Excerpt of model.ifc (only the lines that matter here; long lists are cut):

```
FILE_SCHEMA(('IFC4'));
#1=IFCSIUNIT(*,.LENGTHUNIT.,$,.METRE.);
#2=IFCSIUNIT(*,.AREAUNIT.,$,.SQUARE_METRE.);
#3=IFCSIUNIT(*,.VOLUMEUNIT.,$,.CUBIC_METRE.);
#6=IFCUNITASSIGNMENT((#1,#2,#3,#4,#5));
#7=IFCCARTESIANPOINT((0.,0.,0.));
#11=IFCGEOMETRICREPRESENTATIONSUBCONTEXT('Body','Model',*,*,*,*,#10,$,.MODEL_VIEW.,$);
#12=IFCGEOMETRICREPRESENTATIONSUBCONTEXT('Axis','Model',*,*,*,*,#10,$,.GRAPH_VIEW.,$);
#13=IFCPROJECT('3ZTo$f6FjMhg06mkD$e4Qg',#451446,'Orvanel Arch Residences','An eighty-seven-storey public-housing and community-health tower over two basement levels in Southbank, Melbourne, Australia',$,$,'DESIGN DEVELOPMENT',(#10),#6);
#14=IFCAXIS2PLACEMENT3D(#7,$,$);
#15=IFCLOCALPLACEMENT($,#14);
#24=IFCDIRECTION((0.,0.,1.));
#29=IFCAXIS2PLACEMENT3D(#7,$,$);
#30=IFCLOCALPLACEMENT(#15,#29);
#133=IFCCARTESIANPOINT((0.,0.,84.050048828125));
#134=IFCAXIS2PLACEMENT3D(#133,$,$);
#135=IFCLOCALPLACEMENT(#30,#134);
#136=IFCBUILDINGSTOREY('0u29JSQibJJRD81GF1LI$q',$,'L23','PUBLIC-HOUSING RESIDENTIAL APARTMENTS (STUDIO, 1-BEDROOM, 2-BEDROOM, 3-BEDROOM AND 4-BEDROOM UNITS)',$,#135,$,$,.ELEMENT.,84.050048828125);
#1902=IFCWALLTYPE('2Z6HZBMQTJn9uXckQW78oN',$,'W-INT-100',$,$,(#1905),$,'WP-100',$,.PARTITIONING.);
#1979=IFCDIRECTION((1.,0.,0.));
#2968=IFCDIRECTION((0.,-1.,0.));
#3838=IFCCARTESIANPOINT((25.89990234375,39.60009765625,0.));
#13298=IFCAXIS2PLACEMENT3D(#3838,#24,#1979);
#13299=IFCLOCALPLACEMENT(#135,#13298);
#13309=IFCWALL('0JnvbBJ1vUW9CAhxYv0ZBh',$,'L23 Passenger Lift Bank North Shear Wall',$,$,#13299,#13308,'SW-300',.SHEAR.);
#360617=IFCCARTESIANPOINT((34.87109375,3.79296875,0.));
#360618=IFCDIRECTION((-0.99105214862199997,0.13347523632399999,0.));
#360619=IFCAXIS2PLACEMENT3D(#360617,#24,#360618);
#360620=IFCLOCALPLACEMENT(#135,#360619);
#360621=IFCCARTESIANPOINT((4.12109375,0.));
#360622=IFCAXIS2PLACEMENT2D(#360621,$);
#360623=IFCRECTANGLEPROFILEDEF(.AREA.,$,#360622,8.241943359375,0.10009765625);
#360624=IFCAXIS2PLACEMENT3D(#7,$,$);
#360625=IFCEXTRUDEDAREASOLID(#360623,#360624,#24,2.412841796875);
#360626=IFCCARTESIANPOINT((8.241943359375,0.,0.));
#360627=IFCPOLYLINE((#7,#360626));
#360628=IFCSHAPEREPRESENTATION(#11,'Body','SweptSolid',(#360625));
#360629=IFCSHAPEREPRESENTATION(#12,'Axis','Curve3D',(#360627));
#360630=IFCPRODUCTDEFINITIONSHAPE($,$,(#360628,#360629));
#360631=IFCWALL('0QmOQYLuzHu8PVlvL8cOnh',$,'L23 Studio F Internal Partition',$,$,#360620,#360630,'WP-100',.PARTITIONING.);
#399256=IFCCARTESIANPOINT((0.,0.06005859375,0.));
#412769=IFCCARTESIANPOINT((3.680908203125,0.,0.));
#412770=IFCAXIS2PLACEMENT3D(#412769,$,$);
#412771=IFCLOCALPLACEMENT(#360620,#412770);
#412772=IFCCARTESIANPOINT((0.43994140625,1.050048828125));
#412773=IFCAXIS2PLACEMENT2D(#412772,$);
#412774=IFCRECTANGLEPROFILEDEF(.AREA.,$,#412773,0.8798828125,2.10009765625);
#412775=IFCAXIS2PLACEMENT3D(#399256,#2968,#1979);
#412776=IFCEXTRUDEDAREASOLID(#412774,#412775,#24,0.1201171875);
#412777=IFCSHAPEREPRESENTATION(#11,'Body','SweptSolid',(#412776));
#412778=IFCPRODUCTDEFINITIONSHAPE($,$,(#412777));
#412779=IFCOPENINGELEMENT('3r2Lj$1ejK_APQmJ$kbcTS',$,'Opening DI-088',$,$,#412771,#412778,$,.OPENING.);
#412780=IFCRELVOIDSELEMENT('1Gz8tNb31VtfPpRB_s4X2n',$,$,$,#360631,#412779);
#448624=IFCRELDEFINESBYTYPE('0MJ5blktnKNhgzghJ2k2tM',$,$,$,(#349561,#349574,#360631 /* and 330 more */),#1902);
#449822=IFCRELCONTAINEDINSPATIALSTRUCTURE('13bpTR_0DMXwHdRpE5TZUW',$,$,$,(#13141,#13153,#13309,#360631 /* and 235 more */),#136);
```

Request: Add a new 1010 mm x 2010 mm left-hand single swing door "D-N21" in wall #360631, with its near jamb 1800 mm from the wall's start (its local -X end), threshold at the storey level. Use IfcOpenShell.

```python
import numpy as np
import ifcopenshell
import ifcopenshell.api.feature
import ifcopenshell.api.geometry
import ifcopenshell.api.root
import ifcopenshell.api.spatial
import ifcopenshell.geom
import ifcopenshell.util.element
import ifcopenshell.util.placement
import ifcopenshell.util.representation
import ifcopenshell.util.shape
import ifcopenshell.util.unit

model = ifcopenshell.open("model.ifc")
unit_scale = ifcopenshell.util.unit.calculate_unit_scale(model)
settings = ifcopenshell.geom.settings()


def volume(element):
    """Net volume in cubic metres, openings subtracted."""
    shape = ifcopenshell.geom.create_shape(settings, element)
    return ifcopenshell.util.shape.get_volume(shape.geometry)


wall = model.by_guid("0QmOQYLuzHu8PVlvL8cOnh")
storey = ifcopenshell.util.element.get_container(wall, ifc_class="IfcBuildingStorey")
context = ifcopenshell.util.representation.get_context(model, "Model", "Body", "MODEL_VIEW")
before = volume(wall)

width, height, from_end, sill = 1.01, 2.01, 1.8, 0.0  # metres

# The wall runs along its own X axis, and the end named is its -X end.
wall_shape = ifcopenshell.geom.create_shape(settings, wall)
x, y, z = ifcopenshell.util.shape.get_vertices(wall_shape.geometry).T
start = x.min() + from_end
face, thickness = float(y.min()), float(y.max() - y.min())
wall_matrix = ifcopenshell.util.placement.get_local_placement(wall.ObjectPlacement)
level = ifcopenshell.util.placement.get_local_placement(storey.ObjectPlacement)[2, 3]


def in_wall(x, y):
    """Placement at x, y metres in the wall's axes, at sill height."""
    matrix = wall_matrix.copy()
    matrix[:, 3] = wall_matrix @ np.array([x / unit_scale, y / unit_scale, 0.0, 1.0])
    matrix[2, 3] = level + sill / unit_scale
    return matrix


# Opening: a box that overshoots both wall faces by 50 mm.
opening = ifcopenshell.api.root.create_entity(model, ifc_class="IfcOpeningElement", predefined_type="OPENING")
box = ifcopenshell.api.geometry.add_wall_representation(
    model, context=context, length=width, height=height, thickness=thickness + 0.1
)
ifcopenshell.api.geometry.assign_representation(model, product=opening, representation=box)
ifcopenshell.api.geometry.edit_object_placement(model, product=opening, matrix=in_wall(start, face - 0.05), is_si=False)
ifcopenshell.api.feature.add_feature(model, feature=opening, element=wall)

door = ifcopenshell.api.root.create_entity(model, ifc_class="IfcDoor", name="D-N21", predefined_type="DOOR")
door.OverallWidth, door.OverallHeight = width / unit_scale, height / unit_scale
door.OperationType = "SINGLE_SWING_LEFT"
body = ifcopenshell.api.geometry.add_door_representation(
    model,
    context=context,
    overall_width=door.OverallWidth,
    overall_height=door.OverallHeight,
    operation_type="SINGLE_SWING_LEFT",
    lining_properties={"LiningDepth": thickness / unit_scale, "ThresholdDepth": thickness / unit_scale},
)
ifcopenshell.api.geometry.assign_representation(model, product=door, representation=body)
ifcopenshell.api.spatial.assign_container(model, products=[door], relating_structure=storey)
ifcopenshell.api.feature.add_filling(model, opening=opening, element=door)

# The lining spans the wall, so the door starts at the wall face.
ifcopenshell.api.geometry.edit_object_placement(model, product=door, matrix=in_wall(start, face), is_si=False)

after = volume(wall)

print(f"wall volume {before:.3f} -> {after:.3f} m3")

model.write("model_updated.ifc")
```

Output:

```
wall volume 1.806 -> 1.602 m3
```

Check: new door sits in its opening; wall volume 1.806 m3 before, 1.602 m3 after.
